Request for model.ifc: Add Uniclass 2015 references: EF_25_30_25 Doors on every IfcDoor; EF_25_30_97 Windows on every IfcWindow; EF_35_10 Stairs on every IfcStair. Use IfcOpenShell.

First a look at what the model holds.

```python
import ifcopenshell

model = ifcopenshell.open("model.ifc")
print(model.schema)
print("classifications:", [c.Name for c in model.by_type("IfcClassification")])
for ifc_class in ("IfcDoor", "IfcRoof", "IfcStair", "IfcWall", "IfcWindow"):
    print(ifc_class, len(model.by_type(ifc_class)))
```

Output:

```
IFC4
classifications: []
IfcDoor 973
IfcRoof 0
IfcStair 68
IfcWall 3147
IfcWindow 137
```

```python
import ifcopenshell
import ifcopenshell.api.classification

model = ifcopenshell.open("model.ifc")

system = ifcopenshell.api.classification.add_classification(model, classification="Uniclass 2015")

codes = {
    "IfcDoor": ("EF_25_30_25", "Doors"),
    "IfcWindow": ("EF_25_30_97", "Windows"),
    "IfcStair": ("EF_35_10", "Stairs"),
}
for ifc_class, (code, name) in codes.items():
    products = model.by_type(ifc_class)
    ifcopenshell.api.classification.add_reference(
        model, products=products, classification=system, identification=code, name=name
    )
    print(code, len(products))

model.write("model_v2.ifc")
```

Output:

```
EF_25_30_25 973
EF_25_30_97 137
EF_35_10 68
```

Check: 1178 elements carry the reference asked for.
